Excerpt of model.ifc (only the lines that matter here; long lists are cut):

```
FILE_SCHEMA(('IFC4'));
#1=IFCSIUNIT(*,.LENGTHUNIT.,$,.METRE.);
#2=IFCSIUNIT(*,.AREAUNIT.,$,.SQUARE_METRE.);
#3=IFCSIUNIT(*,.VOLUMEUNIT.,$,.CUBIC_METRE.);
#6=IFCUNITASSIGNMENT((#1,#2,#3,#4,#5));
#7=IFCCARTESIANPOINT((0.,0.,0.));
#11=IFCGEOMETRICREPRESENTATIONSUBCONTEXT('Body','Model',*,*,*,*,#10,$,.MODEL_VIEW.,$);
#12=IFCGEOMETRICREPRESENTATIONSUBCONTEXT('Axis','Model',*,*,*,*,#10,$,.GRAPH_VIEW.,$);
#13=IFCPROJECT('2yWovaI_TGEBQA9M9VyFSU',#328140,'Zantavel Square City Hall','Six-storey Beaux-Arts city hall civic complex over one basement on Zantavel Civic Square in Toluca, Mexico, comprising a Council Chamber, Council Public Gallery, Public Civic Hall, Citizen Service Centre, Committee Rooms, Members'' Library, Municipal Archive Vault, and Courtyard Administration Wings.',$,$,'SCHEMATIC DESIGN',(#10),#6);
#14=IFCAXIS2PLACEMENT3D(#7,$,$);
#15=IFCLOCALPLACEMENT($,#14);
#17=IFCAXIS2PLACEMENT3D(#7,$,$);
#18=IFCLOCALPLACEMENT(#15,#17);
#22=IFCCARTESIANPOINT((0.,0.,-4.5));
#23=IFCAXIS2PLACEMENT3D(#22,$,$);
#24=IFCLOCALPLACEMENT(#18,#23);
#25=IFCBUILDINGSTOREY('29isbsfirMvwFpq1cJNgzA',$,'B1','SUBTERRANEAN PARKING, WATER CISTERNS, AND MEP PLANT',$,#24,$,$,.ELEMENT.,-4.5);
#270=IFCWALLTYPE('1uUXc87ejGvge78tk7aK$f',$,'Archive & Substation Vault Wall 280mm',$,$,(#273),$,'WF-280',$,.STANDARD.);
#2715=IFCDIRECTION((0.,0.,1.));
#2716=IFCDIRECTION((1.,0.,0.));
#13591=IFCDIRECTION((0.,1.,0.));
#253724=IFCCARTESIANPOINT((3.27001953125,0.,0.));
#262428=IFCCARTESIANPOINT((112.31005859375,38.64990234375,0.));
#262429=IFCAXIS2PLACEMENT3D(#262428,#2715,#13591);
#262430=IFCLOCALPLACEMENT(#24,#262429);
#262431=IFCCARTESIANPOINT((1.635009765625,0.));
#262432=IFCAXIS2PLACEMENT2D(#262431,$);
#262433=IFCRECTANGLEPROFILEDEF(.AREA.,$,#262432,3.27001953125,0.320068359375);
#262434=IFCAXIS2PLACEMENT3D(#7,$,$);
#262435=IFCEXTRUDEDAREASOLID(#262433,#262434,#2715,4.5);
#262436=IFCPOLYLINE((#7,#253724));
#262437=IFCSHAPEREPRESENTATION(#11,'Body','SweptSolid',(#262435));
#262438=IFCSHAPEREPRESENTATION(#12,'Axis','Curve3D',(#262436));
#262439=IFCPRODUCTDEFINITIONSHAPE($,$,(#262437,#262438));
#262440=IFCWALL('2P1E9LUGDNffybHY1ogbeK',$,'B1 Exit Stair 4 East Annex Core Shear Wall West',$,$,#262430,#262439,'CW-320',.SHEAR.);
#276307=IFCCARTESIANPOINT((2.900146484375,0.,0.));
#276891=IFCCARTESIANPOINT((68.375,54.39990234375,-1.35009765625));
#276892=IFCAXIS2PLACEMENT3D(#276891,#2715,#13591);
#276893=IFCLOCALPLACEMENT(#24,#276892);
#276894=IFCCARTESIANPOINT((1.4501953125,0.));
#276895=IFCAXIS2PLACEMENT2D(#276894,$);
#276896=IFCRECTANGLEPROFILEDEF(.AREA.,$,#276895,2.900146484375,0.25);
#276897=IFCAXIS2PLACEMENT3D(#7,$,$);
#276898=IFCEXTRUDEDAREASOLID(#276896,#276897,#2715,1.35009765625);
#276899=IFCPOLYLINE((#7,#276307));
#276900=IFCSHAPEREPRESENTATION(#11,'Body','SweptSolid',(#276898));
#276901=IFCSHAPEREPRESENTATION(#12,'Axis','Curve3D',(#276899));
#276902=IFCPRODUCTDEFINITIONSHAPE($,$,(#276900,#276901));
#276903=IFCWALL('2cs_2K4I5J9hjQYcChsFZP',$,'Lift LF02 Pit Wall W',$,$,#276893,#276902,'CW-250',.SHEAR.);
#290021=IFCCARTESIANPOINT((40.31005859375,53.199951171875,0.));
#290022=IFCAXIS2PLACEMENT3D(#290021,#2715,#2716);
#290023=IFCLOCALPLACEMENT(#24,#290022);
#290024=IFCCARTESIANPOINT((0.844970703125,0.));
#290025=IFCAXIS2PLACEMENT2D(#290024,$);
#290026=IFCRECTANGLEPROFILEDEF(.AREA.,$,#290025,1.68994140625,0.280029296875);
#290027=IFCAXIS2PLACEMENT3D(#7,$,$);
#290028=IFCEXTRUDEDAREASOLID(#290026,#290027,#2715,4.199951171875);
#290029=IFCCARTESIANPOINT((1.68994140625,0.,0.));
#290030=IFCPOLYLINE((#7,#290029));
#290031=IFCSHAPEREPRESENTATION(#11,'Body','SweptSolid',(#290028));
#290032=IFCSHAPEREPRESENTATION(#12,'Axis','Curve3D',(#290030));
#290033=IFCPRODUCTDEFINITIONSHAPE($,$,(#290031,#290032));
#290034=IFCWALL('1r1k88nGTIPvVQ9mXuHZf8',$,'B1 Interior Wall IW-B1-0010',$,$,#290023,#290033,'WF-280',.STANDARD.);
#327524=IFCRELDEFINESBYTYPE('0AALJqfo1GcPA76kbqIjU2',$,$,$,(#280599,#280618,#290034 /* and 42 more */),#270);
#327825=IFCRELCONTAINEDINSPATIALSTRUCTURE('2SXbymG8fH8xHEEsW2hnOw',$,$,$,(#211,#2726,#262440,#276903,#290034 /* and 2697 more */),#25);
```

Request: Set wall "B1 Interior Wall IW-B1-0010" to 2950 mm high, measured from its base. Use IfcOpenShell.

```python
import ifcopenshell
import ifcopenshell.geom
import ifcopenshell.util.representation
import ifcopenshell.util.shape

model = ifcopenshell.open("model.ifc")
settings = ifcopenshell.geom.settings()


def volume(element):
    """Net volume in cubic metres, openings subtracted."""
    shape = ifcopenshell.geom.create_shape(settings, element)
    return ifcopenshell.util.shape.get_volume(shape.geometry)


wall = model.by_id(290034)
before = volume(wall)

body = ifcopenshell.util.representation.get_representation(wall, "Model", "Body")
solid = body.Items[0]
old_height = solid.Depth
solid.Depth = 2.95
after = volume(wall)

print(f"height {old_height:g} -> {solid.Depth:g}, volume {before:.3f} -> {after:.3f} m3")

model.write("model-out.ifc")
```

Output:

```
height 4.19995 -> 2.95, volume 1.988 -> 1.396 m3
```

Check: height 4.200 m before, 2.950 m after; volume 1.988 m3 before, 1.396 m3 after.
